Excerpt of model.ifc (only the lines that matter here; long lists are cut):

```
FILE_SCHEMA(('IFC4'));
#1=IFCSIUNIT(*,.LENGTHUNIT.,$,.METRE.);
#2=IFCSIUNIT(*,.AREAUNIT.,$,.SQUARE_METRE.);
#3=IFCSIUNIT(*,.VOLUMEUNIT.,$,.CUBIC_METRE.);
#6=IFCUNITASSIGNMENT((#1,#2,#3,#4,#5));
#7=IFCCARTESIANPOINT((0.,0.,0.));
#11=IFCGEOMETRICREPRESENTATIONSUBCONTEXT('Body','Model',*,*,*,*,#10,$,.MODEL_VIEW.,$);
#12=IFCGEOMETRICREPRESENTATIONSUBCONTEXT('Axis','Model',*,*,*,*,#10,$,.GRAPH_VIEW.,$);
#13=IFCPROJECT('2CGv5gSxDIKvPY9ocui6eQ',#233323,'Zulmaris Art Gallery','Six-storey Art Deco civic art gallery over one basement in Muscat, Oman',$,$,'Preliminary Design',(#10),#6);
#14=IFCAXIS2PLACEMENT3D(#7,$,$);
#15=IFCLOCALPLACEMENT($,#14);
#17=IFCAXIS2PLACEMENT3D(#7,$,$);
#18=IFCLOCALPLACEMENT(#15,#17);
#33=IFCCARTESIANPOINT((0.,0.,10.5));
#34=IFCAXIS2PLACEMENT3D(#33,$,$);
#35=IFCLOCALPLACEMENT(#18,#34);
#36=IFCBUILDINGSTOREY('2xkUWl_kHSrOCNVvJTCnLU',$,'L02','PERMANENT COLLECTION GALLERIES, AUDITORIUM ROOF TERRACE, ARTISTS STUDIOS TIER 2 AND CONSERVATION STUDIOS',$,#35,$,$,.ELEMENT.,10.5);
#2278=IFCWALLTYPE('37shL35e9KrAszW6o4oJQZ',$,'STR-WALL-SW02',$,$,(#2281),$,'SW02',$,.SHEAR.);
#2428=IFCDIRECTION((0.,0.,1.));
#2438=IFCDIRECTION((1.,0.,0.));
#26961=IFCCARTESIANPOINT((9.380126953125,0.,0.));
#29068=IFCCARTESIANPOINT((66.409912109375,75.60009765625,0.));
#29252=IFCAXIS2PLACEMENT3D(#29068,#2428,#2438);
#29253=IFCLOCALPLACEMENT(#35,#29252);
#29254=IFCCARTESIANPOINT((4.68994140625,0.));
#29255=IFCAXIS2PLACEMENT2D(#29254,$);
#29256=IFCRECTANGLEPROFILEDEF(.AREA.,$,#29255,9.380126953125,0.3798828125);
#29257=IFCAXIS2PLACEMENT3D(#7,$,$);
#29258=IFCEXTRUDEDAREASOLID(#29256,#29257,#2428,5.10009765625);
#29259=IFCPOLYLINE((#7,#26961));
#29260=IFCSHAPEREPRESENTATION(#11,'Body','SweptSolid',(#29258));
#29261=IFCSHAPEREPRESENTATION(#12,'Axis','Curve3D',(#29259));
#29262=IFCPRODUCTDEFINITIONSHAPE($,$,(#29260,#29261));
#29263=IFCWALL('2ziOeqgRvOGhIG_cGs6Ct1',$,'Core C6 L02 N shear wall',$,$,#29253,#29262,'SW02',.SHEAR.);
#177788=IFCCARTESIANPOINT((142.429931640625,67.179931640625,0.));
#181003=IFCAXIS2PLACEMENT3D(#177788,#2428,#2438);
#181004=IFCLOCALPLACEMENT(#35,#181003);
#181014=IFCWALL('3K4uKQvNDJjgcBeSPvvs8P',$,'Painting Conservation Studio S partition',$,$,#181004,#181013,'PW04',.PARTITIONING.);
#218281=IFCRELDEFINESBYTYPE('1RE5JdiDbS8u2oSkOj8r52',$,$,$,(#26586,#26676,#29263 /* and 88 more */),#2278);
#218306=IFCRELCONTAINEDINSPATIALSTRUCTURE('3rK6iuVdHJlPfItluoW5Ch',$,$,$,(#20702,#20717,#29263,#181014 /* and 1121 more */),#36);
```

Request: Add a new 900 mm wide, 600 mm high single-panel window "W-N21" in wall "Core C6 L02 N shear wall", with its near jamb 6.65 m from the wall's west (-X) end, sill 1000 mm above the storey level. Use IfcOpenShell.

```python
import numpy as np
import ifcopenshell
import ifcopenshell.api.feature
import ifcopenshell.api.geometry
import ifcopenshell.api.root
import ifcopenshell.api.spatial
import ifcopenshell.geom
import ifcopenshell.util.element
import ifcopenshell.util.placement
import ifcopenshell.util.representation
import ifcopenshell.util.shape
import ifcopenshell.util.unit

model = ifcopenshell.open("model.ifc")
unit_scale = ifcopenshell.util.unit.calculate_unit_scale(model)
settings = ifcopenshell.geom.settings()


def volume(element):
    """Net volume in cubic metres, openings subtracted."""
    shape = ifcopenshell.geom.create_shape(settings, element)
    return ifcopenshell.util.shape.get_volume(shape.geometry)


wall = model.by_guid("2ziOeqgRvOGhIG_cGs6Ct1")
storey = ifcopenshell.util.element.get_container(wall, ifc_class="IfcBuildingStorey")
context = ifcopenshell.util.representation.get_context(model, "Model", "Body", "MODEL_VIEW")
before = volume(wall)

width, height, from_end, sill = 0.9, 0.6, 6.65, 1  # metres

# The wall runs along its own X axis, and the end named is its -X end.
wall_shape = ifcopenshell.geom.create_shape(settings, wall)
x, y, z = ifcopenshell.util.shape.get_vertices(wall_shape.geometry).T
start = x.min() + from_end
face, thickness = float(y.min()), float(y.max() - y.min())
wall_matrix = ifcopenshell.util.placement.get_local_placement(wall.ObjectPlacement)
level = ifcopenshell.util.placement.get_local_placement(storey.ObjectPlacement)[2, 3]


def in_wall(x, y):
    """Placement at x, y metres in the wall's axes, at sill height."""
    matrix = wall_matrix.copy()
    matrix[:, 3] = wall_matrix @ np.array([x / unit_scale, y / unit_scale, 0.0, 1.0])
    matrix[2, 3] = level + sill / unit_scale
    return matrix


# Opening: a box that overshoots both wall faces by 50 mm.
opening = ifcopenshell.api.root.create_entity(model, ifc_class="IfcOpeningElement", predefined_type="OPENING")
box = ifcopenshell.api.geometry.add_wall_representation(
    model, context=context, length=width, height=height, thickness=thickness + 0.1
)
ifcopenshell.api.geometry.assign_representation(model, product=opening, representation=box)
ifcopenshell.api.geometry.edit_object_placement(model, product=opening, matrix=in_wall(start, face - 0.05), is_si=False)
ifcopenshell.api.feature.add_feature(model, feature=opening, element=wall)

window = ifcopenshell.api.root.create_entity(model, ifc_class="IfcWindow", name="W-N21", predefined_type="WINDOW")
window.OverallWidth, window.OverallHeight = width / unit_scale, height / unit_scale
window.PartitioningType = "SINGLE_PANEL"
body = ifcopenshell.api.geometry.add_window_representation(
    model,
    context=context,
    overall_width=window.OverallWidth,
    overall_height=window.OverallHeight,
    partition_type="SINGLE_PANEL",
)
ifcopenshell.api.geometry.assign_representation(model, product=window, representation=body)
ifcopenshell.api.spatial.assign_container(model, products=[window], relating_structure=storey)
ifcopenshell.api.feature.add_filling(model, opening=opening, element=window)

# Centre the window in the wall's thickness.
ifcopenshell.api.geometry.edit_object_placement(model, product=window, matrix=in_wall(start, face), is_si=False)
window_shape = ifcopenshell.geom.create_shape(settings, window)
depth = ifcopenshell.util.shape.get_vertices(window_shape.geometry)[:, 1]
offset = face + thickness / 2 - (depth.min() + depth.max()) / 2
ifcopenshell.api.geometry.edit_object_placement(model, product=window, matrix=in_wall(start, offset), is_si=False)

after = volume(wall)

print(f"wall volume {before:.3f} -> {after:.3f} m3")

model.write("model-out.ifc")
```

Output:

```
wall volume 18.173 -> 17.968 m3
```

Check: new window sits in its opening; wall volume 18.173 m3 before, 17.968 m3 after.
